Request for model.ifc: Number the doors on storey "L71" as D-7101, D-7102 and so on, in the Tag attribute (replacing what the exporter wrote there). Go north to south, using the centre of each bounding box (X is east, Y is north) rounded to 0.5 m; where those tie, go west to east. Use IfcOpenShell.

First a look at what the model holds.

```python
import ifcopenshell
import ifcopenshell.util.element
import ifcopenshell.util.placement

model = ifcopenshell.open("model.ifc")
print(model.schema)
storey = next(s for s in model.by_type("IfcBuildingStorey") if s.Name == "L71")
doors = [e for e in ifcopenshell.util.element.get_decomposition(storey) if e.is_a("IfcDoor")]
for e in sorted(doors, key=lambda e: e.id()):
    origin = ifcopenshell.util.placement.get_local_placement(e.ObjectPlacement)[:3, 3]
    print(e.id(), e.Tag, e.Name, origin.round(2) + 0.0, sep=" | ")
```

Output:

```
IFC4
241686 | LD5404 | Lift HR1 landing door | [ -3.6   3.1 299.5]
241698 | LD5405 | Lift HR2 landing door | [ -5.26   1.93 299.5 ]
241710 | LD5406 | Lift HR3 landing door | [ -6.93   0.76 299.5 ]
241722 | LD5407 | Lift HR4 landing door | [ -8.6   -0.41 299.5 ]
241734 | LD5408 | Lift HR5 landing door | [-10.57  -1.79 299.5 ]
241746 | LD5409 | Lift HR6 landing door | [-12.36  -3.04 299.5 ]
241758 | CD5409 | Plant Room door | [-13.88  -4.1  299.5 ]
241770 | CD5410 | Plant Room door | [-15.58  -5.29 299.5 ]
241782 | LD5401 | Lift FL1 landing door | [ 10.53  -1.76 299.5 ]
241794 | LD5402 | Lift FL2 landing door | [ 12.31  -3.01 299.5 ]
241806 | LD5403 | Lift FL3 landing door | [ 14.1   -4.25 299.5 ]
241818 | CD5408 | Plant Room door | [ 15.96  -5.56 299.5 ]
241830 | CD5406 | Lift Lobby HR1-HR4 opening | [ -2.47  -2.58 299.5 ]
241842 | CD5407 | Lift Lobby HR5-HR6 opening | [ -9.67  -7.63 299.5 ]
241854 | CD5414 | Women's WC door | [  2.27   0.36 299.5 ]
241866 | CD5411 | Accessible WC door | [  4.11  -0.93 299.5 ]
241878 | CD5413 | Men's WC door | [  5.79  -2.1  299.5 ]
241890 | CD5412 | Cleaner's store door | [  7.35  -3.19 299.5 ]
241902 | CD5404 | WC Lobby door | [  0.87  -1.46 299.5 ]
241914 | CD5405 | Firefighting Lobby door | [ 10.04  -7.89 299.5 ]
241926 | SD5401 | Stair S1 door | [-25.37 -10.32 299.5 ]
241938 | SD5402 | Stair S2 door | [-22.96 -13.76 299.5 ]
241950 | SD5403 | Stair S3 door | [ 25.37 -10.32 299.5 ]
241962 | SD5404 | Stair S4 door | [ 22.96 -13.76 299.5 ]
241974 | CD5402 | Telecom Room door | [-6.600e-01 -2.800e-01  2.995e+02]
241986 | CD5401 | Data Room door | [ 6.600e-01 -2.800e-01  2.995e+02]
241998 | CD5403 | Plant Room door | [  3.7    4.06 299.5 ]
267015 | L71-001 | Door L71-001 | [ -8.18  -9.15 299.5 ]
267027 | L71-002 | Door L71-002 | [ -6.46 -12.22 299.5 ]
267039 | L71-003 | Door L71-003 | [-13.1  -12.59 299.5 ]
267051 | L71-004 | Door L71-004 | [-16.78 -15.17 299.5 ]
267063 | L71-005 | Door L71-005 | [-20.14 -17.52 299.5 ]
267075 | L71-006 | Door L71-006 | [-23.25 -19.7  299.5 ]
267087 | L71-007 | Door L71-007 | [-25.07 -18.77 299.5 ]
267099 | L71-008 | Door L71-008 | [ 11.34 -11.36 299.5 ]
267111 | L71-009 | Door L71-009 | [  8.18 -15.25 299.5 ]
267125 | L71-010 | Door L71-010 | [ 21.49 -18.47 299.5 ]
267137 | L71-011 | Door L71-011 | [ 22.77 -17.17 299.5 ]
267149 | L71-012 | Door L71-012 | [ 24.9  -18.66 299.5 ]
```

```python
import ifcopenshell
import ifcopenshell.geom
import ifcopenshell.util.element
import ifcopenshell.util.shape

model = ifcopenshell.open("model.ifc")
settings = ifcopenshell.geom.settings()
settings.set("use-world-coords", True)


def centre(element):
    shape = ifcopenshell.geom.create_shape(settings, element)
    return ifcopenshell.util.shape.get_bbox_centroid(shape.geometry)


storey = next(s for s in model.by_type("IfcBuildingStorey") if s.Name == "L71")
doors = [e for e in ifcopenshell.util.element.get_decomposition(storey) if e.is_a("IfcDoor")]

# Insertion points can sit at a corner or the storey origin, so sort by the geometry (in metres).
centres = {e: centre(e) for e in doors}
doors.sort(key=lambda e: (-round(centres[e][1] / 0.5), centres[e][0]))

for i, e in enumerate(doors, start=1):
    number = f"D-71{i:02d}"
    e.Tag = number
    print(e.id(), number)

model.write("model_rev.ifc")
```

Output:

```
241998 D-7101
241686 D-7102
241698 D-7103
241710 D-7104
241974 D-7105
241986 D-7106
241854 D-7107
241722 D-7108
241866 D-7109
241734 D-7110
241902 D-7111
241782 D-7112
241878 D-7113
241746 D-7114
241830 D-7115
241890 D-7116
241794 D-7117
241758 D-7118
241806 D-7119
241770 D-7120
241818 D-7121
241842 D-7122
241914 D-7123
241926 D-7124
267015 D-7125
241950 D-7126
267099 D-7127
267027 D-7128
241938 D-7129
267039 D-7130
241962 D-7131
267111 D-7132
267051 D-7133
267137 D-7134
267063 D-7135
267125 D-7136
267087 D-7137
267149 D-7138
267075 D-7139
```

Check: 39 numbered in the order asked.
